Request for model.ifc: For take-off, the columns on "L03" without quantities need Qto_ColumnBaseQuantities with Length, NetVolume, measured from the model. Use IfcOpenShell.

First a look at what the model holds.

```python
import ifcopenshell
import ifcopenshell.util.element
import ifcopenshell.util.unit

model = ifcopenshell.open("model.ifc")
print(model.schema)
for unit_type in ("LENGTHUNIT", "AREAUNIT", "VOLUMEUNIT"):
    print(unit_type, ifcopenshell.util.unit.calculate_unit_scale(model, unit_type))
storey = next(s for s in model.by_type("IfcBuildingStorey") if s.Name == "L03")
columns = [e for e in ifcopenshell.util.element.get_decomposition(storey) if e.is_a("IfcColumn")]
for e in sorted(columns, key=lambda e: e.id()):
    print(e.id(), e.is_a(), e.Name, list(ifcopenshell.util.element.get_psets(e, qtos_only=True)), sep=" | ")
```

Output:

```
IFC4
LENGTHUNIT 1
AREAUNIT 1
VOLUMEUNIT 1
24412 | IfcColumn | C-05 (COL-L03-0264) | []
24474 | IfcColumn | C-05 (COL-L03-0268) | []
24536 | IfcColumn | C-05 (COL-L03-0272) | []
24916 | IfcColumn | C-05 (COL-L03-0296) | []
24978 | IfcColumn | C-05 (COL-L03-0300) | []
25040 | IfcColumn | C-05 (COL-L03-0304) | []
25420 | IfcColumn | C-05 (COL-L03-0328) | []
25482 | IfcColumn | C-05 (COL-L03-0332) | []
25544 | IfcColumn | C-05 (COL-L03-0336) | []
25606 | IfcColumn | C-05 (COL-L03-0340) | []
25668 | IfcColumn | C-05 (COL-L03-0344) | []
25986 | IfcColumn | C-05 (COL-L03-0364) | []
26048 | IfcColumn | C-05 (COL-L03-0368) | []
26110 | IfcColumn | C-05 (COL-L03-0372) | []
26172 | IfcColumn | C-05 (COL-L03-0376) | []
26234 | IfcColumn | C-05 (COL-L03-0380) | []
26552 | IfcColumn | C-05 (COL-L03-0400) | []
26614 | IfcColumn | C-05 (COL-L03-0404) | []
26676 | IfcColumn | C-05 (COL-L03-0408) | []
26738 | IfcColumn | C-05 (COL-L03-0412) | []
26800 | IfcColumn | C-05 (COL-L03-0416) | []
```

```python
import ifcopenshell
import ifcopenshell.api.pset
import ifcopenshell.geom
import ifcopenshell.util.element
import ifcopenshell.util.shape
import ifcopenshell.util.unit

model = ifcopenshell.open("model.ifc")
unit_scale = ifcopenshell.util.unit.calculate_unit_scale(model)
volume_scale = ifcopenshell.util.unit.calculate_unit_scale(model, "VOLUMEUNIT")
settings = ifcopenshell.geom.settings()

storey = next(s for s in model.by_type("IfcBuildingStorey") if s.Name == "L03")
columns = [e for e in ifcopenshell.util.element.get_decomposition(storey) if e.is_a("IfcColumn")]

for e in sorted(columns, key=lambda e: e.id()):
    if ifcopenshell.util.element.get_psets(e, qtos_only=True, should_inherit=False):
        continue
    # Geometry comes back in metres, in the element's own axes.
    shape = ifcopenshell.geom.create_shape(settings, e)
    values = {
        "Length": ifcopenshell.util.shape.get_z(shape.geometry) / unit_scale,
        "NetVolume": ifcopenshell.util.shape.get_volume(shape.geometry) / volume_scale,
    }
    qto = ifcopenshell.api.pset.add_qto(model, product=e, name="Qto_ColumnBaseQuantities")
    ifcopenshell.api.pset.edit_qto(model, qto=qto, properties=values)
    print(e.id(), {k: round(v, 3) for k, v in values.items()})

model.write("model-out.ifc")
```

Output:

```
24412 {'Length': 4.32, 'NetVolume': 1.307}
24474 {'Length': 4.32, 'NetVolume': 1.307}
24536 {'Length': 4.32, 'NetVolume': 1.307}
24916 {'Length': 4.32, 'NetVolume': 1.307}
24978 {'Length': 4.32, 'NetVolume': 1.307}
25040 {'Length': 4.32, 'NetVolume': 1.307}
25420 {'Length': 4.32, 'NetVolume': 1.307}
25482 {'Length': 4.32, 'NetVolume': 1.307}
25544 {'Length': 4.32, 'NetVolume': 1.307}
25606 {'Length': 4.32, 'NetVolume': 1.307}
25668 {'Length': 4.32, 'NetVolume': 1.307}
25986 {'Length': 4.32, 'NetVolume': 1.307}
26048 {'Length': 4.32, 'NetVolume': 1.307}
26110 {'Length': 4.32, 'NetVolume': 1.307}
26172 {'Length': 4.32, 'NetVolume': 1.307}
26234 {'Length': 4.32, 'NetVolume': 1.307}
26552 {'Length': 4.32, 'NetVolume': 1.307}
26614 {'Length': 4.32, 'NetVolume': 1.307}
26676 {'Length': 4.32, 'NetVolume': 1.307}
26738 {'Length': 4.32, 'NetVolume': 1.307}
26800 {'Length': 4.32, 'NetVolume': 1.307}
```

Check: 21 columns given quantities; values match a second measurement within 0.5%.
